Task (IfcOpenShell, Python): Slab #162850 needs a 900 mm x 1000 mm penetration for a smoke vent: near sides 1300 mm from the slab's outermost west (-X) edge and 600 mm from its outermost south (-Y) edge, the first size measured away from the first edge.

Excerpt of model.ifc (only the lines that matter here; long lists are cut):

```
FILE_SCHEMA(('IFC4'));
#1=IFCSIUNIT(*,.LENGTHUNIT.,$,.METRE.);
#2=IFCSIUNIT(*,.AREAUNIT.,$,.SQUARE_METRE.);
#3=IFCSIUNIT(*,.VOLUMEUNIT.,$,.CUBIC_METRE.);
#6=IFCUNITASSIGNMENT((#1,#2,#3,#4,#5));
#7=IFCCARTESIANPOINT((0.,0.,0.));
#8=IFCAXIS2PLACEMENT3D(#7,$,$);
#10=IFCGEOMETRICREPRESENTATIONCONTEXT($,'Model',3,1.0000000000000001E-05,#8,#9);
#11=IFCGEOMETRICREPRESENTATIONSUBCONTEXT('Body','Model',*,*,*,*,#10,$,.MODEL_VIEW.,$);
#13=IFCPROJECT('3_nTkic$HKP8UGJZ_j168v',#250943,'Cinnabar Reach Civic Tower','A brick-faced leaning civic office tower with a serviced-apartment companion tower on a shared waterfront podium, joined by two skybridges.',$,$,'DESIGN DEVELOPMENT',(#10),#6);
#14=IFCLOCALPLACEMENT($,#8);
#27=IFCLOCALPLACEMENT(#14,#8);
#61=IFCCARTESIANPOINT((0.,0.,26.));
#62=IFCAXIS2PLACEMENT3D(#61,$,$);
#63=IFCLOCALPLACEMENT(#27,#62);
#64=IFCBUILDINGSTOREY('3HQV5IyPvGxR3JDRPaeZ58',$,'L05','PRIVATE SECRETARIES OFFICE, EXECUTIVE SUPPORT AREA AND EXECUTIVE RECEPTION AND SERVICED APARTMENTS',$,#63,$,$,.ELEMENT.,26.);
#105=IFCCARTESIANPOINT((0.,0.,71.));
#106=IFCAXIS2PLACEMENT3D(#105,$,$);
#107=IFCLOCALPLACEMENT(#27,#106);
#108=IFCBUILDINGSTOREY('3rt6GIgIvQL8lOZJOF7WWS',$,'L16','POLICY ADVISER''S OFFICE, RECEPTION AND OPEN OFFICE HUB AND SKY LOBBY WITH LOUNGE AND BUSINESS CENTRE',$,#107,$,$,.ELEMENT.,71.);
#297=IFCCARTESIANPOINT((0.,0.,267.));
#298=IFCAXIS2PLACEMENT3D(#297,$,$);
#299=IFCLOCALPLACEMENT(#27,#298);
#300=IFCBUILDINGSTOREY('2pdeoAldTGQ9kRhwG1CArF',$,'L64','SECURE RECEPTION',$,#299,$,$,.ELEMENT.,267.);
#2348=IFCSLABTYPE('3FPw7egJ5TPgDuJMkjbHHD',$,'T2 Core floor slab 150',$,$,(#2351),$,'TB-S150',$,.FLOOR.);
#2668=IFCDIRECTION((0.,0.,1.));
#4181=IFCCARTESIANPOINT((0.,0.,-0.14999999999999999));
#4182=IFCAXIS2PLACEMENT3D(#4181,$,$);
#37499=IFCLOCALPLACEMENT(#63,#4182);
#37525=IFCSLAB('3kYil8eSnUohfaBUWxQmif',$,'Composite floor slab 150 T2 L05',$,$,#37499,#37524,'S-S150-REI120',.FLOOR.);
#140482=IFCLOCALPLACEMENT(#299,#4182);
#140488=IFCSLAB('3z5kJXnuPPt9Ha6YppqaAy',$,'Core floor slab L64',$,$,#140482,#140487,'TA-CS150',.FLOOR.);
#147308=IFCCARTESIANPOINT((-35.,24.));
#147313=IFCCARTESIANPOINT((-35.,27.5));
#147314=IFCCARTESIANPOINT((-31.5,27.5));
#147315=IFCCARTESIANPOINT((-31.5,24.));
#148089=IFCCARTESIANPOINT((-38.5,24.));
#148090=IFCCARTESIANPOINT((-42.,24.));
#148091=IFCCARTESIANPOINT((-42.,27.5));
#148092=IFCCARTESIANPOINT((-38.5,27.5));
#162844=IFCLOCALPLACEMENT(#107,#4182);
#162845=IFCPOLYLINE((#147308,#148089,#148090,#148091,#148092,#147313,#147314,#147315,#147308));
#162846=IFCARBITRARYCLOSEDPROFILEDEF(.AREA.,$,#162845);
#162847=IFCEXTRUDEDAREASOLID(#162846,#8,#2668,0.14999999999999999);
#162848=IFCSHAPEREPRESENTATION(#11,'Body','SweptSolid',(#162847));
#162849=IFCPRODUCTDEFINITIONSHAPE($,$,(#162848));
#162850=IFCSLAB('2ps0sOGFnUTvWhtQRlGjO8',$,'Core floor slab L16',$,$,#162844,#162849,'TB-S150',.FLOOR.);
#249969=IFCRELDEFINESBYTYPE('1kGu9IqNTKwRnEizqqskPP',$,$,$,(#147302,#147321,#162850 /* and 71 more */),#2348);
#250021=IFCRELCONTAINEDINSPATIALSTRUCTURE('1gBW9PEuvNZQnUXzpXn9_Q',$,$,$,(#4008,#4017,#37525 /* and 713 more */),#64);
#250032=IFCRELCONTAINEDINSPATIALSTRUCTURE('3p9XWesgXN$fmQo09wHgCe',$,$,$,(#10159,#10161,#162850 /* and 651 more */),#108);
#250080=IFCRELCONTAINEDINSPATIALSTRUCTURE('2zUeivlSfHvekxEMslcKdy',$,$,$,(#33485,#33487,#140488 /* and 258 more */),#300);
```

```python
import numpy as np
import ifcopenshell
import ifcopenshell.api.feature
import ifcopenshell.api.geometry
import ifcopenshell.api.root
import ifcopenshell.geom
import ifcopenshell.util.placement
import ifcopenshell.util.representation
import ifcopenshell.util.shape
import ifcopenshell.util.unit

model = ifcopenshell.open("model.ifc")
unit_scale = ifcopenshell.util.unit.calculate_unit_scale(model)
settings = ifcopenshell.geom.settings()


def volume(element):
    """Net volume in cubic metres, openings subtracted."""
    shape = ifcopenshell.geom.create_shape(settings, element)
    return ifcopenshell.util.shape.get_volume(shape.geometry)


slab = model.by_guid("2ps0sOGFnUTvWhtQRlGjO8")
before = volume(slab)

# Extent in the slab's own axes, in metres. The edges named are its -X and -Y sides.
slab_shape = ifcopenshell.geom.create_shape(settings, slab)
vertices = ifcopenshell.util.shape.get_vertices(slab_shape.geometry)
x_min, y_min, bottom = vertices.min(axis=0)
top = vertices[:, 2].max()

opening = ifcopenshell.api.root.create_entity(model, ifc_class="IfcOpeningElement", name="Smoke vent opening", predefined_type="OPENING")
context = ifcopenshell.util.representation.get_context(model, "Model", "Body", "MODEL_VIEW")
width, depth = 0.9, 1
outline = [(0.0, 0.0), (width, 0.0), (width, depth), (0.0, depth), (0.0, 0.0)]
# Overshoot both faces by 50 mm so the cut is clean.
shape = ifcopenshell.api.geometry.add_slab_representation(
    model, context=context, depth=top - bottom + 0.1, polyline=outline
)
ifcopenshell.api.geometry.assign_representation(model, product=opening, representation=shape)

matrix = ifcopenshell.util.placement.get_local_placement(slab.ObjectPlacement)
matrix[:, 3] = matrix @ np.append(np.array([x_min + 1.3, y_min + 0.6, bottom - 0.05]) / unit_scale, 1.0)
ifcopenshell.api.geometry.edit_object_placement(model, product=opening, matrix=matrix, is_si=False)
ifcopenshell.api.feature.add_feature(model, feature=opening, element=slab)

after = volume(slab)

print(f"slab volume {before:.3f} -> {after:.3f} m3")

model.write("model_edited.ifc")
```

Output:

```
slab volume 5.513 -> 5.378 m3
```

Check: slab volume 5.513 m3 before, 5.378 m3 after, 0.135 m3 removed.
